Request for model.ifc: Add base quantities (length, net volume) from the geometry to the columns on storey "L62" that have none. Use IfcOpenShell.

First a look at what the model holds.

```python
import ifcopenshell
import ifcopenshell.util.element
import ifcopenshell.util.unit

model = ifcopenshell.open("model.ifc")
print(model.schema)
for unit_type in ("LENGTHUNIT", "AREAUNIT", "VOLUMEUNIT"):
    print(unit_type, ifcopenshell.util.unit.calculate_unit_scale(model, unit_type))
storey = next(s for s in model.by_type("IfcBuildingStorey") if s.Name == "L62")
columns = [e for e in ifcopenshell.util.element.get_decomposition(storey) if e.is_a("IfcColumn")]
for e in sorted(columns, key=lambda e: e.id()):
    print(e.id(), e.is_a(), e.Name, list(ifcopenshell.util.element.get_psets(e, qtos_only=True)), sep=" | ")
```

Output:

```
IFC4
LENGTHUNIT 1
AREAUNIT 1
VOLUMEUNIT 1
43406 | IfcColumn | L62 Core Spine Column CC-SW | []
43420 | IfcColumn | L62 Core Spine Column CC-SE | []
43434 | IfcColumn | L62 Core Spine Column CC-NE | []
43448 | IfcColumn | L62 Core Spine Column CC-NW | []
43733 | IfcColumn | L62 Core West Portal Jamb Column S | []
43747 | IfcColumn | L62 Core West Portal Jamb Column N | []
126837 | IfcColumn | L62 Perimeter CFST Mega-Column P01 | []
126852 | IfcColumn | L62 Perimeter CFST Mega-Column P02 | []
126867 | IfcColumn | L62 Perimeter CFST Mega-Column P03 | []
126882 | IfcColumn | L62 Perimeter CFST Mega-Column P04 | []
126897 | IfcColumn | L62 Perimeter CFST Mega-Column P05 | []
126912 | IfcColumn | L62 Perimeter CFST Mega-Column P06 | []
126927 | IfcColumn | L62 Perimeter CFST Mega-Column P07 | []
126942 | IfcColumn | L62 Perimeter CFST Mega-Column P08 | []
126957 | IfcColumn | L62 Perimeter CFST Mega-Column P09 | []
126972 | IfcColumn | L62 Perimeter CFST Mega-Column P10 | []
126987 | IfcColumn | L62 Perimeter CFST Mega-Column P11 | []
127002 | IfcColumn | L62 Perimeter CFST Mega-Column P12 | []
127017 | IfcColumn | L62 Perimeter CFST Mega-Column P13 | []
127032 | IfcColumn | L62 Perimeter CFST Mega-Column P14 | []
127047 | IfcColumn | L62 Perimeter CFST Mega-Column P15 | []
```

```python
import ifcopenshell
import ifcopenshell.api.pset
import ifcopenshell.geom
import ifcopenshell.util.element
import ifcopenshell.util.shape
import ifcopenshell.util.unit

model = ifcopenshell.open("model.ifc")
unit_scale = ifcopenshell.util.unit.calculate_unit_scale(model)
volume_scale = ifcopenshell.util.unit.calculate_unit_scale(model, "VOLUMEUNIT")
settings = ifcopenshell.geom.settings()

storey = next(s for s in model.by_type("IfcBuildingStorey") if s.Name == "L62")
columns = [e for e in ifcopenshell.util.element.get_decomposition(storey) if e.is_a("IfcColumn")]

for e in sorted(columns, key=lambda e: e.id()):
    if ifcopenshell.util.element.get_psets(e, qtos_only=True, should_inherit=False):
        continue
    # Geometry comes back in metres, in the element's own axes.
    shape = ifcopenshell.geom.create_shape(settings, e)
    values = {
        "Length": ifcopenshell.util.shape.get_z(shape.geometry) / unit_scale,
        "NetVolume": ifcopenshell.util.shape.get_volume(shape.geometry) / volume_scale,
    }
    qto = ifcopenshell.api.pset.add_qto(model, product=e, name="Qto_ColumnBaseQuantities")
    ifcopenshell.api.pset.edit_qto(model, qto=qto, properties=values)
    print(e.id(), {k: round(v, 3) for k, v in values.items()})

model.write("model_rev.ifc")
```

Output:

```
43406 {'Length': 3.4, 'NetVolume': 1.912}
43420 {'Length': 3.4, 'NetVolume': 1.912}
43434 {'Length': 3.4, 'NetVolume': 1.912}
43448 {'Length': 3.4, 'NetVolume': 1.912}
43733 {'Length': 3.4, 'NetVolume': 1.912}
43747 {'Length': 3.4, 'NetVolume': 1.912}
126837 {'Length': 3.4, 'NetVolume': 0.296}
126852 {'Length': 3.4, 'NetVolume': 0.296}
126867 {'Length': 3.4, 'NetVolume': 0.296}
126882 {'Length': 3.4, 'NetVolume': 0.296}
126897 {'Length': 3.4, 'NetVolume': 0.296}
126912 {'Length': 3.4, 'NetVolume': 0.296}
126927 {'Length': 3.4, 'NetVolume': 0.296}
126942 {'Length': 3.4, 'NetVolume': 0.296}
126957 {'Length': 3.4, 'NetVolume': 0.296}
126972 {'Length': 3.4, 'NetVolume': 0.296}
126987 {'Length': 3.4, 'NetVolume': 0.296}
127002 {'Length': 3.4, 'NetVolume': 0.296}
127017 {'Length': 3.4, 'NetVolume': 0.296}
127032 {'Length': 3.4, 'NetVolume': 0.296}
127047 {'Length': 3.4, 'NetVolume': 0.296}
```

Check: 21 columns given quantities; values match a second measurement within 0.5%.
